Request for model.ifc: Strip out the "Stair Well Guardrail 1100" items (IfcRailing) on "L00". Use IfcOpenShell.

First a look at what the model holds.

```python
import ifcopenshell
import ifcopenshell.util.element

model = ifcopenshell.open("model.ifc")
print(model.schema)
storey = next(s for s in model.by_type("IfcBuildingStorey") if s.Name == "L00")
railings = [e for e in ifcopenshell.util.element.get_decomposition(storey) if e.is_a("IfcRailing")]
seen = {}
for e in railings:
    element_type = ifcopenshell.util.element.get_type(e)
    name = element_type.Name if element_type not in (None, e) else None
    seen[name] = seen.get(name, 0) + 1
for name, count in sorted(seen.items(), key=str):
    print(count, "x", name)
```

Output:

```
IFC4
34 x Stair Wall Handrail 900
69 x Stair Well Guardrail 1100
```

```python
import ifcopenshell
import ifcopenshell.api.root
import ifcopenshell.util.element

model = ifcopenshell.open("model.ifc")

storey = next(s for s in model.by_type("IfcBuildingStorey") if s.Name == "L00")
railings = [e for e in ifcopenshell.util.element.get_decomposition(storey) if e.is_a("IfcRailing")]
targets = [e for e in railings if (t := ifcopenshell.util.element.get_type(e)) not in (None, e) and t.Name == "Stair Well Guardrail 1100"]

for e in targets:
    ifcopenshell.api.root.remove_product(model, product=e)
print(len(targets), "removed")

model.write("model-out.ifc")
```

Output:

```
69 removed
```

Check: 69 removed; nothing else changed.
